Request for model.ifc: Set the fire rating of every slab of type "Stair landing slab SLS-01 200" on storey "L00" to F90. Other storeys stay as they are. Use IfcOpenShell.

First a look at what the model holds.

```python
import ifcopenshell
import ifcopenshell.util.element

model = ifcopenshell.open("model.ifc")
print(model.schema)
storey = next(s for s in model.by_type("IfcBuildingStorey") if s.Name == "L00")
slabs = [e for e in ifcopenshell.util.element.get_decomposition(storey) if e.is_a("IfcSlab")]
seen = {}
for e in slabs:
    element_type = ifcopenshell.util.element.get_type(e)
    key = (element_type.Name if element_type != e and element_type else None, ifcopenshell.util.element.get_pset(e, "Pset_SlabCommon", "FireRating"))
    seen[key] = seen.get(key, 0) + 1
for (name, value), count in sorted(seen.items(), key=str):
    print(count, "x", name, "|", value)
```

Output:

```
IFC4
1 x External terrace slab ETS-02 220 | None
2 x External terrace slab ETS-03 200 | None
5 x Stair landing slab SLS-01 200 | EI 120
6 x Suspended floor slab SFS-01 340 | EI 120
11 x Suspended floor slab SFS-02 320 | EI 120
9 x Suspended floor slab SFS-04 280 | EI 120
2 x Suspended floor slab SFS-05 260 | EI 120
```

```python
import ifcopenshell
import ifcopenshell.api.pset
import ifcopenshell.util.element

model = ifcopenshell.open("model.ifc")

storey = next(s for s in model.by_type("IfcBuildingStorey") if s.Name == "L00")
slabs = [e for e in ifcopenshell.util.element.get_decomposition(storey) if e.is_a("IfcSlab")]

count = 0
for e in slabs:
    element_type = ifcopenshell.util.element.get_type(e)
    if element_type in (None, e) or element_type.Name != "Stair landing slab SLS-01 200":
        continue
    # add_pset returns the element's existing set when there is one.
    pset = ifcopenshell.api.pset.add_pset(model, product=e, name="Pset_SlabCommon")
    ifcopenshell.api.pset.edit_pset(model, pset=pset, properties={"FireRating": "F90"})
    count += 1

print(count, "slabs updated")

model.write("model_v2.ifc")
```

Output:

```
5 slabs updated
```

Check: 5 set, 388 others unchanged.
